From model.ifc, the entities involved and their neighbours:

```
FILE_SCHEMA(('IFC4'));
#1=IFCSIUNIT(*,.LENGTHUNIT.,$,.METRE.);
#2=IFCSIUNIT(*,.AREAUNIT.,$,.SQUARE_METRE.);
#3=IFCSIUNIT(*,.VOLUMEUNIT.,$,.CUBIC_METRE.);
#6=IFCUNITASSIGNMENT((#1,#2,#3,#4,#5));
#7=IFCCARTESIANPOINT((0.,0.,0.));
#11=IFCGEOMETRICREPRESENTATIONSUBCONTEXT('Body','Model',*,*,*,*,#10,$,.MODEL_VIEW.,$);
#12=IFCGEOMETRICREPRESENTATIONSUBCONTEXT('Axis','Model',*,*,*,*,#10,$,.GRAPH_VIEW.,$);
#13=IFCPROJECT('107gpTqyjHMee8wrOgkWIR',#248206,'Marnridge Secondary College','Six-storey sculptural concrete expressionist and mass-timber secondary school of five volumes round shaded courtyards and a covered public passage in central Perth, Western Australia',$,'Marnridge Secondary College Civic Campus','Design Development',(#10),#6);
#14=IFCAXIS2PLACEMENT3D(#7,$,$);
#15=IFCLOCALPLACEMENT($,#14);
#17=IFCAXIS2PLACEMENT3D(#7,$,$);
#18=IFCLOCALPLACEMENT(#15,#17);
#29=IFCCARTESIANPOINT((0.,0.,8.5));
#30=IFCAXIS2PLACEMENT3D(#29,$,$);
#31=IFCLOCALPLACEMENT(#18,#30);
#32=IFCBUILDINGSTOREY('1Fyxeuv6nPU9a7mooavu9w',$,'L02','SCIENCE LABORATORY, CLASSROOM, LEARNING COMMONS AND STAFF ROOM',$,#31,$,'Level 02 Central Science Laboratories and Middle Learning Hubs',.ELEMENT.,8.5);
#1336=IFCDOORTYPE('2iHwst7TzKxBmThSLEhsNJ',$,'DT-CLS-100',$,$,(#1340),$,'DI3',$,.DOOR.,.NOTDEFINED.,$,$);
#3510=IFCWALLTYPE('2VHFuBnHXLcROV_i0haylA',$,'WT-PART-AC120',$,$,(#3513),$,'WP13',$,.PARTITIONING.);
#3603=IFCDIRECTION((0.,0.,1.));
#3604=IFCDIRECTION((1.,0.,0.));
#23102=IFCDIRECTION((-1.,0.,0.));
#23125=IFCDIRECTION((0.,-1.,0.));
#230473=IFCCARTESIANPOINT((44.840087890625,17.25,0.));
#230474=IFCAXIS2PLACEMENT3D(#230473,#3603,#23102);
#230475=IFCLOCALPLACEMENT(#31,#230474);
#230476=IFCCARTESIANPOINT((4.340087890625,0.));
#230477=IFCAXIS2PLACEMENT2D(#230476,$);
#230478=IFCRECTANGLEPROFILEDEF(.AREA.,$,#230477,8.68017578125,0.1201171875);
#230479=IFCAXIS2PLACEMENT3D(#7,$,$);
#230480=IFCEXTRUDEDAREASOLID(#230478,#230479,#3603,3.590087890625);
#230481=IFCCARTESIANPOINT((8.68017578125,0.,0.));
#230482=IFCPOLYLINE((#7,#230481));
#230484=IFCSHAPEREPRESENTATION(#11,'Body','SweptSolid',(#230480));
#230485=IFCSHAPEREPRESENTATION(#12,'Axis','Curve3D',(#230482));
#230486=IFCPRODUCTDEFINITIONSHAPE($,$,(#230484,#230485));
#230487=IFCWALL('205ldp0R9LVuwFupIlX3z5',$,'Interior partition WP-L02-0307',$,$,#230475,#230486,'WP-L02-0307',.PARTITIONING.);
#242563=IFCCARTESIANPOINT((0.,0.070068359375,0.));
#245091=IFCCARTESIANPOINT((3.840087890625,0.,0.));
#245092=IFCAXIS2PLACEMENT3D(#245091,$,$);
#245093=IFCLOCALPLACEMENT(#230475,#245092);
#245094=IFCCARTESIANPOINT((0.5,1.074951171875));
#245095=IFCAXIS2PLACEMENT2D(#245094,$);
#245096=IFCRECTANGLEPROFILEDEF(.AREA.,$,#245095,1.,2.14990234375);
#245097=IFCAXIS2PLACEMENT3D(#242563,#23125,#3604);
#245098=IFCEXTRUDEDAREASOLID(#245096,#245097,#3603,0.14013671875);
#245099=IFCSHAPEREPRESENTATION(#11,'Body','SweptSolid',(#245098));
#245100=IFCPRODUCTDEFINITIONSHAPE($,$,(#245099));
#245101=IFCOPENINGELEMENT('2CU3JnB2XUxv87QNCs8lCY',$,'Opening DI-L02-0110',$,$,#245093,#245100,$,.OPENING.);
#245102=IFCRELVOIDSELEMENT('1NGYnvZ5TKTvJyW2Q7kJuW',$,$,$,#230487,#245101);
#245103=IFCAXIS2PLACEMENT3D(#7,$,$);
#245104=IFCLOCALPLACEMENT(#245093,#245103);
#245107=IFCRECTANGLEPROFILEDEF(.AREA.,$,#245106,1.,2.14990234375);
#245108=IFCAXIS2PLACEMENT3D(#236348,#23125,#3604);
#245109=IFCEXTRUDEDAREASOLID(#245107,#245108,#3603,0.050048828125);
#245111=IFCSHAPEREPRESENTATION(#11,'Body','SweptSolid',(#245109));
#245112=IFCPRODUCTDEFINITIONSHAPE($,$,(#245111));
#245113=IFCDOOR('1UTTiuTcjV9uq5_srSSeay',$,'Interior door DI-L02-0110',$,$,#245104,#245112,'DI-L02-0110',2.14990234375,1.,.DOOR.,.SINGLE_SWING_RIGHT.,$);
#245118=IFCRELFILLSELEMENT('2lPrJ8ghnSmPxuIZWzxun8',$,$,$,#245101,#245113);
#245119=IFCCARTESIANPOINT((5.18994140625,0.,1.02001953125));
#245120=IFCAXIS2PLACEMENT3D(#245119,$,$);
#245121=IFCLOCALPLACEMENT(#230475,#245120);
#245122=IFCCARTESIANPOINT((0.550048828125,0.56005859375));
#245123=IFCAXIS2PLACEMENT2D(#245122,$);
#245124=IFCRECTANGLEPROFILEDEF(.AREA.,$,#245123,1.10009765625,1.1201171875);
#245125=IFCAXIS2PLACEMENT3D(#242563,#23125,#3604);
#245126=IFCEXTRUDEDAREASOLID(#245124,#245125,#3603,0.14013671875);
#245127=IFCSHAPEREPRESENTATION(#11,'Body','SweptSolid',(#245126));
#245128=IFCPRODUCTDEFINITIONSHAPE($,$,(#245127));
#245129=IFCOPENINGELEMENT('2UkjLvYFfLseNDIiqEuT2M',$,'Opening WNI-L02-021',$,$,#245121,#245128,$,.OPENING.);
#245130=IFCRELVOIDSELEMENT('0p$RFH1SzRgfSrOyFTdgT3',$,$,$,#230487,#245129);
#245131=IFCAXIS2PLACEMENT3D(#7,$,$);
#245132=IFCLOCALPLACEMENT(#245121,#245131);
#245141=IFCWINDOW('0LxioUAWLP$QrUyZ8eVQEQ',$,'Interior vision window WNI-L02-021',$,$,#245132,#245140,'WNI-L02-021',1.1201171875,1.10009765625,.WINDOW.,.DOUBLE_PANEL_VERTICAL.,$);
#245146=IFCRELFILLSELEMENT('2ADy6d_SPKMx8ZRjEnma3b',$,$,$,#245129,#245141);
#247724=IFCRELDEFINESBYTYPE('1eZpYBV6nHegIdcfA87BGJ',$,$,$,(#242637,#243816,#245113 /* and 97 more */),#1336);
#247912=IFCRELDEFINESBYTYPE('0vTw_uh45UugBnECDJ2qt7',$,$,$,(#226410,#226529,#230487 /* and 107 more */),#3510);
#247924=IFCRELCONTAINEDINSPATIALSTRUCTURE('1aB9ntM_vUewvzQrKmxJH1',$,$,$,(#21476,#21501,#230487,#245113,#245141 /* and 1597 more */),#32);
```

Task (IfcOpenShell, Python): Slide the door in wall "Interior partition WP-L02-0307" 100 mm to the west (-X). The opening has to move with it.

```python
import ifcopenshell
import ifcopenshell.api.geometry
import ifcopenshell.util.placement

model = ifcopenshell.open("model.ifc")

door = model.by_id(245113)
opening = door.FillsVoids[0].RelatingOpeningElement
wall = opening.VoidsElements[0].RelatingBuildingElement

wall_matrix = ifcopenshell.util.placement.get_local_placement(wall.ObjectPlacement)
shift = wall_matrix[:3, 0] * 0.1
before = ifcopenshell.util.placement.get_local_placement(door.ObjectPlacement)[:3, 3].copy()

# The door is placed relative to its opening, so it follows when the opening moves.
matrix = ifcopenshell.util.placement.get_local_placement(opening.ObjectPlacement)
matrix[:3, 3] += shift
ifcopenshell.api.geometry.edit_object_placement(
    model, product=opening, matrix=matrix, is_si=False, should_transform_children=True
)

after = ifcopenshell.util.placement.get_local_placement(door.ObjectPlacement)[:3, 3]
print("door moved by", (after - before).round(3) + 0.0)

model.write("model_v2.ifc")
```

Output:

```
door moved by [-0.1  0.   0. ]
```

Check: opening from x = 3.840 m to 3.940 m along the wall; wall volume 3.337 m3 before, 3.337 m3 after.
